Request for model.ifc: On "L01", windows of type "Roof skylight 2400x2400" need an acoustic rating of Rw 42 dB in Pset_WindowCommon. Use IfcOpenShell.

First a look at what the model holds.

```python
import ifcopenshell
import ifcopenshell.util.element

model = ifcopenshell.open("model.ifc")
print(model.schema)
storey = next(s for s in model.by_type("IfcBuildingStorey") if s.Name == "L01")
windows = [e for e in ifcopenshell.util.element.get_decomposition(storey) if e.is_a("IfcWindow")]
seen = {}
for e in windows:
    element_type = ifcopenshell.util.element.get_type(e)
    key = (element_type.Name if element_type != e and element_type else None, ifcopenshell.util.element.get_pset(e, "Pset_WindowCommon", "AcousticRating"))
    seen[key] = seen.get(key, 0) + 1
for (name, value), count in sorted(seen.items(), key=str):
    print(count, "x", name, "|", value)
```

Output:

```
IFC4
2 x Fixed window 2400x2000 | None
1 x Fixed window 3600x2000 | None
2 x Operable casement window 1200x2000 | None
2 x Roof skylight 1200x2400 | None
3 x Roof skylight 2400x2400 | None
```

```python
import ifcopenshell
import ifcopenshell.api.pset
import ifcopenshell.util.element

model = ifcopenshell.open("model.ifc")

storey = next(s for s in model.by_type("IfcBuildingStorey") if s.Name == "L01")
windows = [e for e in ifcopenshell.util.element.get_decomposition(storey) if e.is_a("IfcWindow")]

count = 0
for e in windows:
    element_type = ifcopenshell.util.element.get_type(e)
    if element_type in (None, e) or element_type.Name != "Roof skylight 2400x2400":
        continue
    found = ifcopenshell.util.element.get_pset(e, "Pset_WindowCommon", should_inherit=False)
    if found:
        pset = model.by_id(found["id"])
        if len(ifcopenshell.util.element.get_elements_by_pset(pset)) > 1:
            pset = ifcopenshell.api.pset.unshare_pset(model, products=[e], pset=pset)[0]
    else:
        pset = ifcopenshell.api.pset.add_pset(model, product=e, name="Pset_WindowCommon")
    ifcopenshell.api.pset.edit_pset(model, pset=pset, properties={"AcousticRating": "Rw 42 dB"})
    count += 1

print(count, "windows updated")

model.write("model_rev.ifc")
```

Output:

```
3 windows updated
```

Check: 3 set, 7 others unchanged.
